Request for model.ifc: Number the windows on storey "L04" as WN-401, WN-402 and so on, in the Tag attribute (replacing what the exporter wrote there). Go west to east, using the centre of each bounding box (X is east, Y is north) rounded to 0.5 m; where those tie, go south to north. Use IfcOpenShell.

First a look at what the model holds.

```python
import ifcopenshell
import ifcopenshell.util.element
import ifcopenshell.util.placement

model = ifcopenshell.open("model.ifc")
print(model.schema)
storey = next(s for s in model.by_type("IfcBuildingStorey") if s.Name == "L04")
windows = [e for e in ifcopenshell.util.element.get_decomposition(storey) if e.is_a("IfcWindow")]
for e in sorted(windows, key=lambda e: e.id()):
    origin = ifcopenshell.util.placement.get_local_placement(e.ObjectPlacement)[:3, 3]
    print(e.id(), e.Tag, e.Name, origin.round(2) + 0.0, sep=" | ")
```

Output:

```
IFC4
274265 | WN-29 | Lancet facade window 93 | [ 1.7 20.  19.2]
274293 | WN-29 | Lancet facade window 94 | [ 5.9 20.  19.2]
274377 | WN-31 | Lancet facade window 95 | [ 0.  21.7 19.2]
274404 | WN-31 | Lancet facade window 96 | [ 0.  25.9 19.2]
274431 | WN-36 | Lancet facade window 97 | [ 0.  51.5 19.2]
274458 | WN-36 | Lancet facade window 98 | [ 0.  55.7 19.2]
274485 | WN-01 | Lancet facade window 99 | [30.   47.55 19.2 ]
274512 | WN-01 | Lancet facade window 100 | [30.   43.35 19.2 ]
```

```python
import ifcopenshell
import ifcopenshell.geom
import ifcopenshell.util.element
import ifcopenshell.util.shape

model = ifcopenshell.open("model.ifc")
settings = ifcopenshell.geom.settings()
settings.set("use-world-coords", True)


def centre(element):
    shape = ifcopenshell.geom.create_shape(settings, element)
    return ifcopenshell.util.shape.get_bbox_centroid(shape.geometry)


storey = next(s for s in model.by_type("IfcBuildingStorey") if s.Name == "L04")
windows = [e for e in ifcopenshell.util.element.get_decomposition(storey) if e.is_a("IfcWindow")]

# Insertion points can sit at a corner or the storey origin, so sort by the geometry (in metres).
centres = {e: centre(e) for e in windows}
windows.sort(key=lambda e: (round(centres[e][0] / 0.5), centres[e][1]))

for i, e in enumerate(windows, start=1):
    number = f"WN-4{i:02d}"
    e.Tag = number
    print(e.id(), number)

model.write("model_edited.ifc")
```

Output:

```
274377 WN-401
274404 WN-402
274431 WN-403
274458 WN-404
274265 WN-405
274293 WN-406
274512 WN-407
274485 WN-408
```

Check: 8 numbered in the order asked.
